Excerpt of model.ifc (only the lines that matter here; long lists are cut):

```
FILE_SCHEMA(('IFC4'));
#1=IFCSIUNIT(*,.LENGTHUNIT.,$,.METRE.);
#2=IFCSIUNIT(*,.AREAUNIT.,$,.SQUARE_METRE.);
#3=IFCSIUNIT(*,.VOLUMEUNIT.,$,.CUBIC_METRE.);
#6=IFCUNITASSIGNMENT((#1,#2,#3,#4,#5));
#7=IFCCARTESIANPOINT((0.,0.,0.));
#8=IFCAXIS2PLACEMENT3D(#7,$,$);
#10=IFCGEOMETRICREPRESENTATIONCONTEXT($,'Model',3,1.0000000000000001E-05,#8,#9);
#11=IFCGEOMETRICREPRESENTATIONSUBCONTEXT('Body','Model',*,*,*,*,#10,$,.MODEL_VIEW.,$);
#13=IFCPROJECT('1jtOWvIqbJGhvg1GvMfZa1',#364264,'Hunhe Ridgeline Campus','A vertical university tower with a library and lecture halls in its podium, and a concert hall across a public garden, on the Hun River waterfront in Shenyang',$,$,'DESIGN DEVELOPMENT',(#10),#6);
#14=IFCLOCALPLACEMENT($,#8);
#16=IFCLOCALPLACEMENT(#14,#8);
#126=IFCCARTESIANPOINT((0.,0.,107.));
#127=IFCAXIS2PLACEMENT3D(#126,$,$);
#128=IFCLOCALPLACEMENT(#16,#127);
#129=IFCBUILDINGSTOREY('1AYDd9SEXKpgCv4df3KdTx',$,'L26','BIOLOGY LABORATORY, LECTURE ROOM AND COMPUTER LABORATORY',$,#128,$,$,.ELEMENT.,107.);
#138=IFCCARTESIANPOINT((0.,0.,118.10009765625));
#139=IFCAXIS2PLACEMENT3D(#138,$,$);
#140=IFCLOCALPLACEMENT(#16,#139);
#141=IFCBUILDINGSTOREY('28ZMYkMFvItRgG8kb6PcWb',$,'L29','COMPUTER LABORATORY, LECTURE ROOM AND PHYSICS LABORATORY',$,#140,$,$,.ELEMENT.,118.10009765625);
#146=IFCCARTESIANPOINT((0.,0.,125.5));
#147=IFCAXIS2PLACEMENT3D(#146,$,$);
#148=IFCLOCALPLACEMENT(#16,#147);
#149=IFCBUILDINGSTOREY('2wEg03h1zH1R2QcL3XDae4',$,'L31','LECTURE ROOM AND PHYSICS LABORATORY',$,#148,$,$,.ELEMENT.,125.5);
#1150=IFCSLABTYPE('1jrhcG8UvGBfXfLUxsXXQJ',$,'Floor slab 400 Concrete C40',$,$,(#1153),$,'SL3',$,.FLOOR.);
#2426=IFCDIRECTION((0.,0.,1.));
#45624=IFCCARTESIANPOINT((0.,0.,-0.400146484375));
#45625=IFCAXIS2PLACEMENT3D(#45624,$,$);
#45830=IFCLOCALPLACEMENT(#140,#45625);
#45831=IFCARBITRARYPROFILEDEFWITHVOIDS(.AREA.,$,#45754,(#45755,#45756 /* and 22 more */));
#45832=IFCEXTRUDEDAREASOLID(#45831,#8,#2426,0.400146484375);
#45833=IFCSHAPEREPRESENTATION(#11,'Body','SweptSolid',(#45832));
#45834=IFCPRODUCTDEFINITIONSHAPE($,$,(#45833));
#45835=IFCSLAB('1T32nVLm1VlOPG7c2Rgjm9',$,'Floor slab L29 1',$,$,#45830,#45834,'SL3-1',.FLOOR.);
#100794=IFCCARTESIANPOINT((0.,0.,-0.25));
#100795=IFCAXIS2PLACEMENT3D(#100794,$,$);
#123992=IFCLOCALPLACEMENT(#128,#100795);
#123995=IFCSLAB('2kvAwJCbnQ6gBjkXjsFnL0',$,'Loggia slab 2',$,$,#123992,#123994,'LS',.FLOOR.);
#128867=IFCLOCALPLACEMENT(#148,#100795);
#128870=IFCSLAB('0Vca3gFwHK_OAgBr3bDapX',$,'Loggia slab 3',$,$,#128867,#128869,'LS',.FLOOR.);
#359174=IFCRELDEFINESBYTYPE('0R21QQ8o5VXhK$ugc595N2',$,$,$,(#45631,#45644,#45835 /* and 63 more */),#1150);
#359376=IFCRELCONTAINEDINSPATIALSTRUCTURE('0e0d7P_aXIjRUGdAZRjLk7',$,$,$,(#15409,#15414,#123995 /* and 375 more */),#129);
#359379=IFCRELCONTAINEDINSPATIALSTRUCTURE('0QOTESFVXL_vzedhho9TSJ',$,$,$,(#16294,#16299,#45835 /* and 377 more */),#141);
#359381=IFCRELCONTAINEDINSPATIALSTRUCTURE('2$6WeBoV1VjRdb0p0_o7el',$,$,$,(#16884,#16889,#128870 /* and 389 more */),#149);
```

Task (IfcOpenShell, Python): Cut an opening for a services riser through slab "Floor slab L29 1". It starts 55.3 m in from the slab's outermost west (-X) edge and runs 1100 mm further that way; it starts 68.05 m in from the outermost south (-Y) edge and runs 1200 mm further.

```python
import numpy as np
import ifcopenshell
import ifcopenshell.api.feature
import ifcopenshell.api.geometry
import ifcopenshell.api.root
import ifcopenshell.geom
import ifcopenshell.util.placement
import ifcopenshell.util.representation
import ifcopenshell.util.shape
import ifcopenshell.util.unit

model = ifcopenshell.open("model.ifc")
unit_scale = ifcopenshell.util.unit.calculate_unit_scale(model)
settings = ifcopenshell.geom.settings()


def volume(element):
    """Net volume in cubic metres, openings subtracted."""
    shape = ifcopenshell.geom.create_shape(settings, element)
    return ifcopenshell.util.shape.get_volume(shape.geometry)


slab = model.by_guid("1T32nVLm1VlOPG7c2Rgjm9")
before = volume(slab)

# Extent in the slab's own axes, in metres. The edges named are its -X and -Y sides.
slab_shape = ifcopenshell.geom.create_shape(settings, slab)
vertices = ifcopenshell.util.shape.get_vertices(slab_shape.geometry)
x_min, y_min, bottom = vertices.min(axis=0)
top = vertices[:, 2].max()

opening = ifcopenshell.api.root.create_entity(model, ifc_class="IfcOpeningElement", name="Services riser opening", predefined_type="OPENING")
context = ifcopenshell.util.representation.get_context(model, "Model", "Body", "MODEL_VIEW")
width, depth = 1.1, 1.2
outline = [(0.0, 0.0), (width, 0.0), (width, depth), (0.0, depth), (0.0, 0.0)]
# Overshoot both faces by 50 mm so the cut is clean.
shape = ifcopenshell.api.geometry.add_slab_representation(
    model, context=context, depth=top - bottom + 0.1, polyline=outline
)
ifcopenshell.api.geometry.assign_representation(model, product=opening, representation=shape)

matrix = ifcopenshell.util.placement.get_local_placement(slab.ObjectPlacement)
matrix[:, 3] = matrix @ np.append(np.array([x_min + 55.3, y_min + 68.05, bottom - 0.05]) / unit_scale, 1.0)
ifcopenshell.api.geometry.edit_object_placement(model, product=opening, matrix=matrix, is_si=False)
ifcopenshell.api.feature.add_feature(model, feature=opening, element=slab)

after = volume(slab)

print(f"slab volume {before:.3f} -> {after:.3f} m3")

model.write("model_v2.ifc")
```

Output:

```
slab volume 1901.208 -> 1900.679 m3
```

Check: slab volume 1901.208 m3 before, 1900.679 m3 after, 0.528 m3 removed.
